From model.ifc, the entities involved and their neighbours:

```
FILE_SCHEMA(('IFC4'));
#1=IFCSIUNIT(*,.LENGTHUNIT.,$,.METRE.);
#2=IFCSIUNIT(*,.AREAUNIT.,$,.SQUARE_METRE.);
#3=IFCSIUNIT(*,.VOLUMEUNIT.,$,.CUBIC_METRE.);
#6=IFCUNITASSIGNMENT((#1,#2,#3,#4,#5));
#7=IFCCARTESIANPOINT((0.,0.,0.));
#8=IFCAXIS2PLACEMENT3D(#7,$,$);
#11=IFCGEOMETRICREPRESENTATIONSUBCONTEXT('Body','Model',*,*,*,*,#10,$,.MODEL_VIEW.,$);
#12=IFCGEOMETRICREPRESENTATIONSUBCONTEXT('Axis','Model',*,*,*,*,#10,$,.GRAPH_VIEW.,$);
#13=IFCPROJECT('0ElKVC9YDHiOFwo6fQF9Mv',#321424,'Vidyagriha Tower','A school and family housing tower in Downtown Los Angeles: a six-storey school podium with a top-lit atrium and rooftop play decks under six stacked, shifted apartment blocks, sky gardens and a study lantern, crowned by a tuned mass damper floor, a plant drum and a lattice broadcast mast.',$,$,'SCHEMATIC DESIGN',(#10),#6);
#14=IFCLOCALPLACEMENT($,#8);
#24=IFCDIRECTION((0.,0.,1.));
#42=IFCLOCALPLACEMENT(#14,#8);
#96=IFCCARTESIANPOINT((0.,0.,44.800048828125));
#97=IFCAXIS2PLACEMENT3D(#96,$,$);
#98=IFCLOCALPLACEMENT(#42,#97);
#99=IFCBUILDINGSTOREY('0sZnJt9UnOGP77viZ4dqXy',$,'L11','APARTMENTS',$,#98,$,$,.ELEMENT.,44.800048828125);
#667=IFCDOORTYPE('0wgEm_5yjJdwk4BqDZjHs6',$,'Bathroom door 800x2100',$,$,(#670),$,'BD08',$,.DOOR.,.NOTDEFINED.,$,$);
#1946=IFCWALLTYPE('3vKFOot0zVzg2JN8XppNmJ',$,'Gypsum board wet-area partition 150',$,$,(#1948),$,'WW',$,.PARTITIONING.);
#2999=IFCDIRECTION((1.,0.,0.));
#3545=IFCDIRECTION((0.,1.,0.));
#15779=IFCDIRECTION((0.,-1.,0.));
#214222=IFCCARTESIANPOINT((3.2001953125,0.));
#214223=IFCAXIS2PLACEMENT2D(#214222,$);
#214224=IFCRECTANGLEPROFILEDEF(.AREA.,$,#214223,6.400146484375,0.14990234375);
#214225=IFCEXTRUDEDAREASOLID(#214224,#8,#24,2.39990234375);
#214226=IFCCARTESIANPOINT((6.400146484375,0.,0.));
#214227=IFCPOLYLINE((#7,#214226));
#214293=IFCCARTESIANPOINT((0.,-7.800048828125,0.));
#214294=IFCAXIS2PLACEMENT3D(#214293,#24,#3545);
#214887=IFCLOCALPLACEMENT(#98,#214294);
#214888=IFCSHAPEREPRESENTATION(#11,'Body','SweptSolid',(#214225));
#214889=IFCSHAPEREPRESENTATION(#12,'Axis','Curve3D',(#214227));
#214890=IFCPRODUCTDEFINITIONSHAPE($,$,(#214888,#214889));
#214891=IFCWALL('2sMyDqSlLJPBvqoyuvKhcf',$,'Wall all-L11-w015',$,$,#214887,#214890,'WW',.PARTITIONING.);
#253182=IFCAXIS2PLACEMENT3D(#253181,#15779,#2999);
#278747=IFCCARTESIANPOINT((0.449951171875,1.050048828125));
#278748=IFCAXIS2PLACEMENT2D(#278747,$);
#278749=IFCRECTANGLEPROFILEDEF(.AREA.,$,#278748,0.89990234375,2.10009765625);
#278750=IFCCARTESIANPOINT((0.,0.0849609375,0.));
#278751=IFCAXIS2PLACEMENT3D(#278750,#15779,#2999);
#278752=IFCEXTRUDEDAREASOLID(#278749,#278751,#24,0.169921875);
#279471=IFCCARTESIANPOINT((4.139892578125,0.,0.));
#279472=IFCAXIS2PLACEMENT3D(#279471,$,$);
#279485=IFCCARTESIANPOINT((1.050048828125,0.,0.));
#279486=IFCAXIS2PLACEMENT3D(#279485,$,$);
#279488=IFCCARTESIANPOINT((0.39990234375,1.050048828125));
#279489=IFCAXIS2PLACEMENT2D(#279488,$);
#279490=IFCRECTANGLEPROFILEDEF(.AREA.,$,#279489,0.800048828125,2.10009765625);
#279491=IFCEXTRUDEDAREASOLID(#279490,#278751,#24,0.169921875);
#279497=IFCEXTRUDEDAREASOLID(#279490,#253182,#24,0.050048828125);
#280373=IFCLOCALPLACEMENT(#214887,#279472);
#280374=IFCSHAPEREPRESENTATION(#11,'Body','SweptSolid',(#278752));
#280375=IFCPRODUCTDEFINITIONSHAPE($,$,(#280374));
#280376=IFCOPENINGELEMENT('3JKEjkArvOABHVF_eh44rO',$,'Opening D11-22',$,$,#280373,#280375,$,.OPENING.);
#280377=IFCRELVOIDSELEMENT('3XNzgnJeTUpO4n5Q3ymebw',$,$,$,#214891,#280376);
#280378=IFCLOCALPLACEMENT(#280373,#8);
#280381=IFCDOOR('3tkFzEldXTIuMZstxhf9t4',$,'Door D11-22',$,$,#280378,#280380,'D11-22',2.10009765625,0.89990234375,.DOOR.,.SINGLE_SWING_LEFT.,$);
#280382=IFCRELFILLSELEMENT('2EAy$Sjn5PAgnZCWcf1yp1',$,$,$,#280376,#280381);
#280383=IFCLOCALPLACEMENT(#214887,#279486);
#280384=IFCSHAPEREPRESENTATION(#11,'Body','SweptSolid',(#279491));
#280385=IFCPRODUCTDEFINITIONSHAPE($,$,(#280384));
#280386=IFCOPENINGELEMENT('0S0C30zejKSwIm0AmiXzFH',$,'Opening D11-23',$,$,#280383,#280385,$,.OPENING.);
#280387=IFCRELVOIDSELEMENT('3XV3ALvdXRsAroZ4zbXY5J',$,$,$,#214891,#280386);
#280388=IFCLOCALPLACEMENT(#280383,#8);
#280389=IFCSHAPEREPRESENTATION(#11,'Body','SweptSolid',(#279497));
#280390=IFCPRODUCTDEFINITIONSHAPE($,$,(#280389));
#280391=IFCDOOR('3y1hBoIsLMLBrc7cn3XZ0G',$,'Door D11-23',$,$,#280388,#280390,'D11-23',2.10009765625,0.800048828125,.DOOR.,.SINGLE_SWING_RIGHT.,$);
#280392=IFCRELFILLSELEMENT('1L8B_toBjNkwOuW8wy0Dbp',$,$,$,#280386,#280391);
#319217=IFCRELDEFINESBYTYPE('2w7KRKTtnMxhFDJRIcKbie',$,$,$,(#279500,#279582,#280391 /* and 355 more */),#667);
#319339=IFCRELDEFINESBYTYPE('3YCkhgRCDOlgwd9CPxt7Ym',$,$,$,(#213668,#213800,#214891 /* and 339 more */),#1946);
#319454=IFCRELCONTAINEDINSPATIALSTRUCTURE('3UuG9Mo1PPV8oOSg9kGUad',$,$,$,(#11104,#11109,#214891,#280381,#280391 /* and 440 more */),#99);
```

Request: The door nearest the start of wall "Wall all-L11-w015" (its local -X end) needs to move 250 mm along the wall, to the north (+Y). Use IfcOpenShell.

```python
import ifcopenshell
import ifcopenshell.api.geometry
import ifcopenshell.util.placement
import ifcopenshell.util.unit

model = ifcopenshell.open("model.ifc")
unit_scale = ifcopenshell.util.unit.calculate_unit_scale(model)

door = model.by_guid("3y1hBoIsLMLBrc7cn3XZ0G")
opening = door.FillsVoids[0].RelatingOpeningElement
wall = opening.VoidsElements[0].RelatingBuildingElement

wall_matrix = ifcopenshell.util.placement.get_local_placement(wall.ObjectPlacement)
shift = wall_matrix[:3, 0] * 0.25 / unit_scale
before = ifcopenshell.util.placement.get_local_placement(door.ObjectPlacement)[:3, 3].copy()

# The door is placed relative to its opening, so it follows when the opening moves.
matrix = ifcopenshell.util.placement.get_local_placement(opening.ObjectPlacement)
matrix[:3, 3] += shift
ifcopenshell.api.geometry.edit_object_placement(
    model, product=opening, matrix=matrix, is_si=False, should_transform_children=True
)

after = ifcopenshell.util.placement.get_local_placement(door.ObjectPlacement)[:3, 3]
print("door moved by", (after - before).round(3) + 0.0)

model.write("model_v2.ifc")
```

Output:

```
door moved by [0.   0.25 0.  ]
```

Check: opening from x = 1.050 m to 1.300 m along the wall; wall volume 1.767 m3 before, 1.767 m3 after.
